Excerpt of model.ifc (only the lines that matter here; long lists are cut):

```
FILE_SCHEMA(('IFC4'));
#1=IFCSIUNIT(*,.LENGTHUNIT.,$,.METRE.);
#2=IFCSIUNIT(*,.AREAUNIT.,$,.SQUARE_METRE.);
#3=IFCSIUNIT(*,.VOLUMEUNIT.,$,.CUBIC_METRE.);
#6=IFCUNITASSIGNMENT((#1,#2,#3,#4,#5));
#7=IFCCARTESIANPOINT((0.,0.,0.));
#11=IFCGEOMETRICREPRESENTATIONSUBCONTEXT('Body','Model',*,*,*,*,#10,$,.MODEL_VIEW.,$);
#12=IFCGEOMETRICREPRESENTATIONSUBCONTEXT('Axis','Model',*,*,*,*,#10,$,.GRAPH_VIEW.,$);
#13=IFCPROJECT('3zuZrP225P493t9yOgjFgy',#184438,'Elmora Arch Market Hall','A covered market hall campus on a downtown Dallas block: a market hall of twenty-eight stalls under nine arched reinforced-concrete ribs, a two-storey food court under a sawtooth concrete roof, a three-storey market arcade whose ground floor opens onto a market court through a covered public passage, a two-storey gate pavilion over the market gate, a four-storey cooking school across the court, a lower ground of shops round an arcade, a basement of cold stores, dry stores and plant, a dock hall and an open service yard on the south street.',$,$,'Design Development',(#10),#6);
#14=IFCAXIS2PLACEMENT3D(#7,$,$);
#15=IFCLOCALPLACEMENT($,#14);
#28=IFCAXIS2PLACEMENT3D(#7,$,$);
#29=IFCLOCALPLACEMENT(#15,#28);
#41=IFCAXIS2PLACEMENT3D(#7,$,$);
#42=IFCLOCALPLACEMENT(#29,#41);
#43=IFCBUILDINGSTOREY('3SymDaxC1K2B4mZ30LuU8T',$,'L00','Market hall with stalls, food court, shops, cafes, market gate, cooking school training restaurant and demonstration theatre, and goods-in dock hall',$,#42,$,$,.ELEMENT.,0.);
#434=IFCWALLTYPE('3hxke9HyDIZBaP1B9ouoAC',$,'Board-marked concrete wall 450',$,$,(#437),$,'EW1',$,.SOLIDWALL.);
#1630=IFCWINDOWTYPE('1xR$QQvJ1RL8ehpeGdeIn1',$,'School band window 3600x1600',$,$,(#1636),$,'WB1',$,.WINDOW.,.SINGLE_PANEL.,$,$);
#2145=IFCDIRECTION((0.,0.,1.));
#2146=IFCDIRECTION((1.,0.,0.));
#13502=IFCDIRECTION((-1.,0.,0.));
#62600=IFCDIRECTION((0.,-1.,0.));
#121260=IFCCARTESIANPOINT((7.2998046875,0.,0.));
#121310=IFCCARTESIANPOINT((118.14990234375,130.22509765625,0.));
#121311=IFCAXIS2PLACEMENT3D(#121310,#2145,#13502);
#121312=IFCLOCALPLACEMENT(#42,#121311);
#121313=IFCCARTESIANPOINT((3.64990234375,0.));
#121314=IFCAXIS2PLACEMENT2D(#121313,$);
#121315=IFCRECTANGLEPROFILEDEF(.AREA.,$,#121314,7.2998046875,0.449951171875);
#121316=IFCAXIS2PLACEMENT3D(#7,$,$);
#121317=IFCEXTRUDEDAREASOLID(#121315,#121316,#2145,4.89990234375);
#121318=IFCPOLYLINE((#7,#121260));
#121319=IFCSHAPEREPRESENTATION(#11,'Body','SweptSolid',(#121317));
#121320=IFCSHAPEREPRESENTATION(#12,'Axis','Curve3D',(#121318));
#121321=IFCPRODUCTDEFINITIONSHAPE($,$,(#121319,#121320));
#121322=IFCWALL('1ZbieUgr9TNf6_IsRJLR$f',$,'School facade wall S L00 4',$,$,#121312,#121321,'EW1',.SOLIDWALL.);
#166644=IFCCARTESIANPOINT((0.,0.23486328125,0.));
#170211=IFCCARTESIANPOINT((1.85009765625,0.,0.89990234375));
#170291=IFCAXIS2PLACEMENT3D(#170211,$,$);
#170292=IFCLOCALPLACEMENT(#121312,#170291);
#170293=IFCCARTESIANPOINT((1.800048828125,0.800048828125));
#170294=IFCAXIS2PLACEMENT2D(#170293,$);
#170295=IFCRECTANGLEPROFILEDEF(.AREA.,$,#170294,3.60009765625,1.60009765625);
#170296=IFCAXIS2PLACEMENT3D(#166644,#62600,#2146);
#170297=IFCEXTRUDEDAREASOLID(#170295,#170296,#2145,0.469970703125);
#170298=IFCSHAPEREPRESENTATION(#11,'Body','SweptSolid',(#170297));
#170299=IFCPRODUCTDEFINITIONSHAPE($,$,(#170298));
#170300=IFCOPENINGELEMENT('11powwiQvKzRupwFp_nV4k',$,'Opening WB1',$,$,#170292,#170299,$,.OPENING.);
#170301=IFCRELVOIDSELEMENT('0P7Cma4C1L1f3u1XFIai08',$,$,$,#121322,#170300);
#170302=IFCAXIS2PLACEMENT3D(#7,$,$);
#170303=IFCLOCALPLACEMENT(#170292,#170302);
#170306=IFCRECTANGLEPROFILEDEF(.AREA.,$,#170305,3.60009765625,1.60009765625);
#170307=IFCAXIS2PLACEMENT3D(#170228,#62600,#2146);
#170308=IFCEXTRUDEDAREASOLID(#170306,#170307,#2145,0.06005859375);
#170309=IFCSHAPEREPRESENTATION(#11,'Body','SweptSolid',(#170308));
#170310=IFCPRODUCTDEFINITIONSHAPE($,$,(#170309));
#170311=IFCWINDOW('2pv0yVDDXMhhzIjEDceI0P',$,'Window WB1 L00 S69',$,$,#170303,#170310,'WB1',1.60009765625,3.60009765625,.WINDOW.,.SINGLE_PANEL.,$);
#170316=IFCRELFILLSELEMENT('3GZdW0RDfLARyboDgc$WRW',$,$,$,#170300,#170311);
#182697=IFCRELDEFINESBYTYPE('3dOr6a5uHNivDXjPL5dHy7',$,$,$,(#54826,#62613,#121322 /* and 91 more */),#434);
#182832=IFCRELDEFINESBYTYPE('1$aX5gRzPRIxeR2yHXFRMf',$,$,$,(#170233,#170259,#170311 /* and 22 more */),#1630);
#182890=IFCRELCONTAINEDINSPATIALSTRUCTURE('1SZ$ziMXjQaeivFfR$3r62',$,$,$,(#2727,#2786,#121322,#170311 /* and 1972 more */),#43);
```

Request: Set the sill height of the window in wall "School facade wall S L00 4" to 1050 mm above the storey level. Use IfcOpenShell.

```python
import numpy as np
import ifcopenshell
import ifcopenshell.api.geometry
import ifcopenshell.geom
import ifcopenshell.util.element
import ifcopenshell.util.placement
import ifcopenshell.util.shape
import ifcopenshell.util.unit

model = ifcopenshell.open("model.ifc")
unit_scale = ifcopenshell.util.unit.calculate_unit_scale(model)

window = model.by_guid("2pv0yVDDXMhhzIjEDceI0P")
opening = window.FillsVoids[0].RelatingOpeningElement
storey = ifcopenshell.util.element.get_container(window, ifc_class="IfcBuildingStorey")
level = ifcopenshell.util.placement.get_local_placement(storey.ObjectPlacement)[2, 3]

# The opening's origin need not be at the sill, so measure its lowest point.
shape = ifcopenshell.geom.create_shape(ifcopenshell.geom.settings(), opening)
bottom = ifcopenshell.util.shape.get_shape_bottom_elevation(shape, shape.geometry) / unit_scale
dz = level + 1.05 / unit_scale - bottom

shift = np.array([0.0, 0.0, dz])
# The window is placed relative to its opening, so it follows when the opening moves.
matrix = ifcopenshell.util.placement.get_local_placement(opening.ObjectPlacement)
matrix[:3, 3] += shift
ifcopenshell.api.geometry.edit_object_placement(
    model, product=opening, matrix=matrix, is_si=False, should_transform_children=True
)

print(f"moved by {dz * unit_scale:+.3f} m")

model.write("model-out.ifc")
```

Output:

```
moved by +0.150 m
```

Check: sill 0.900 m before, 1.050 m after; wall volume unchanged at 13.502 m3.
